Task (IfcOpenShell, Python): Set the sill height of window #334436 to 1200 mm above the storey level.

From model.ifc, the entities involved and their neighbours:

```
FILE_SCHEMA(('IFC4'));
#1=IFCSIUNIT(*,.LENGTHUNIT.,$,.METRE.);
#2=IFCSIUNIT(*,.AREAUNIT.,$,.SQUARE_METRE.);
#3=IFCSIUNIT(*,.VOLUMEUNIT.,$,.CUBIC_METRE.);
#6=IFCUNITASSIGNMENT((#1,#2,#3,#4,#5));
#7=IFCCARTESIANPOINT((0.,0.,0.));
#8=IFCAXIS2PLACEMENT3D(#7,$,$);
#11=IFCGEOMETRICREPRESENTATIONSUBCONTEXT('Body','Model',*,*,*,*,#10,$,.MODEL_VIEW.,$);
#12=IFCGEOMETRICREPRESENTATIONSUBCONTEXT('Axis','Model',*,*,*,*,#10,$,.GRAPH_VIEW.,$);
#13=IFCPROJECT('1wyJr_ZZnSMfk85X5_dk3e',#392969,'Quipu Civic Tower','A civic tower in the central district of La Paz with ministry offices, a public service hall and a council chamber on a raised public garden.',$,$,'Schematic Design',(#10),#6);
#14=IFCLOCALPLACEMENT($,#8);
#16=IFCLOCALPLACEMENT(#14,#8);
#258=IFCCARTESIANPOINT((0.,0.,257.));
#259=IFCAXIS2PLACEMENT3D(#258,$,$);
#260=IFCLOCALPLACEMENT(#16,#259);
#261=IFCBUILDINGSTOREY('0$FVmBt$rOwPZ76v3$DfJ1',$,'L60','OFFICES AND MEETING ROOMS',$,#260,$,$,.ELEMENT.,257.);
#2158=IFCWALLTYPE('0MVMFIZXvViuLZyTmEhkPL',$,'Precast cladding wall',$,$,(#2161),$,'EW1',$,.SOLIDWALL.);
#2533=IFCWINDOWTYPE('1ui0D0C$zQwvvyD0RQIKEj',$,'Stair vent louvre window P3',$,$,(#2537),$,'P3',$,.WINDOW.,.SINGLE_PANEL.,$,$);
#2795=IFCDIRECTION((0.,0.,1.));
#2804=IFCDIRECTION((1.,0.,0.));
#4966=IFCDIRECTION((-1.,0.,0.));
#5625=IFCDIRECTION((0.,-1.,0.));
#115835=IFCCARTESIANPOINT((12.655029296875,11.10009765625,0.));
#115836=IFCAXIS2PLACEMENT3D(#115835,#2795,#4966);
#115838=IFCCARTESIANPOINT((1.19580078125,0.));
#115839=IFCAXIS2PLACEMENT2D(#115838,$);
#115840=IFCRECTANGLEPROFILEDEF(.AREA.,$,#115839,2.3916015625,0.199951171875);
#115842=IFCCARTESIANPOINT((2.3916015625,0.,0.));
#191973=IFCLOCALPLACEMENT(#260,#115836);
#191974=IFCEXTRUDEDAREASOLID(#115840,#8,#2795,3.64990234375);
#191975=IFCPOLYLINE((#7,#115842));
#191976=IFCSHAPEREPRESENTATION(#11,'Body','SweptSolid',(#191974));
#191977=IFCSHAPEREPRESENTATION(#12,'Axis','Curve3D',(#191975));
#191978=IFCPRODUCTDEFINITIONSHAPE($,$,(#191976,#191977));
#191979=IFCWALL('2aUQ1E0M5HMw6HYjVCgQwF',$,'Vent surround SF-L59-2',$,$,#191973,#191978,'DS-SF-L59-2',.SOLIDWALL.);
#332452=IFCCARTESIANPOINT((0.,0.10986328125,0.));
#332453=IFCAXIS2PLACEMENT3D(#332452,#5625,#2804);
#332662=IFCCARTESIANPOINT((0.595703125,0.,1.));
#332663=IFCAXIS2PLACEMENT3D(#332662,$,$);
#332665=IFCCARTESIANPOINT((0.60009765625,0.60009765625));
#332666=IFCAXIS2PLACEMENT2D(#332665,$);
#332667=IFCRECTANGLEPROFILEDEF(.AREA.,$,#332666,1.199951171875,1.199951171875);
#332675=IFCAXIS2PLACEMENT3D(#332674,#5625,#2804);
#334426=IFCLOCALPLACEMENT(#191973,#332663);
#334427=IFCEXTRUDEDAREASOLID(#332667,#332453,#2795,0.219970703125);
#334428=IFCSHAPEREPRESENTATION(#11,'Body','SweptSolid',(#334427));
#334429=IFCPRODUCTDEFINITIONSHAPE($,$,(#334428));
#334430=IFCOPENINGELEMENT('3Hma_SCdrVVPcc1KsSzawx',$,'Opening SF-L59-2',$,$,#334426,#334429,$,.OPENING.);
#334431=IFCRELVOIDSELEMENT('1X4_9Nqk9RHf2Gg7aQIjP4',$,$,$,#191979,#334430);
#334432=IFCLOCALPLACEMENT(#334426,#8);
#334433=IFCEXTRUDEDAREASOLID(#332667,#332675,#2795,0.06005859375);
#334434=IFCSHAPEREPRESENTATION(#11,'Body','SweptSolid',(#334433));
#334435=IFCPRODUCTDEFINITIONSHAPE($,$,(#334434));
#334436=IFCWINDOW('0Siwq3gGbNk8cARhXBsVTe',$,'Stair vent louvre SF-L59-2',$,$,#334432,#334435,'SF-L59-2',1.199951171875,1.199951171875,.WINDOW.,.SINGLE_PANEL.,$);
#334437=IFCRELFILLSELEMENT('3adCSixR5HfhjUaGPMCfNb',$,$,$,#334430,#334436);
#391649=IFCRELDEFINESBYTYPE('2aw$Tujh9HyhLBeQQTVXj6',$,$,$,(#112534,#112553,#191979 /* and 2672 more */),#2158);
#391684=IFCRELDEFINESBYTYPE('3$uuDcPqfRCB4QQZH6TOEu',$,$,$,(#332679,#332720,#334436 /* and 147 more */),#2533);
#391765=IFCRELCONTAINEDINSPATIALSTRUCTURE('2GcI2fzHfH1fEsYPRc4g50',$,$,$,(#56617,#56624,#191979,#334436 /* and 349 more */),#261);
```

```python
import numpy as np
import ifcopenshell
import ifcopenshell.api.geometry
import ifcopenshell.geom
import ifcopenshell.util.element
import ifcopenshell.util.placement
import ifcopenshell.util.shape
import ifcopenshell.util.unit

model = ifcopenshell.open("model.ifc")
unit_scale = ifcopenshell.util.unit.calculate_unit_scale(model)

window = model.by_guid("0Siwq3gGbNk8cARhXBsVTe")
opening = window.FillsVoids[0].RelatingOpeningElement
storey = ifcopenshell.util.element.get_container(window, ifc_class="IfcBuildingStorey")
level = ifcopenshell.util.placement.get_local_placement(storey.ObjectPlacement)[2, 3]

# The opening's origin need not be at the sill, so measure its lowest point.
shape = ifcopenshell.geom.create_shape(ifcopenshell.geom.settings(), opening)
bottom = ifcopenshell.util.shape.get_shape_bottom_elevation(shape, shape.geometry) / unit_scale
dz = level + 1.2 / unit_scale - bottom

shift = np.array([0.0, 0.0, dz])
# The window is placed relative to its opening, so it follows when the opening moves.
matrix = ifcopenshell.util.placement.get_local_placement(opening.ObjectPlacement)
matrix[:3, 3] += shift
ifcopenshell.api.geometry.edit_object_placement(
    model, product=opening, matrix=matrix, is_si=False, should_transform_children=True
)

print(f"moved by {dz * unit_scale:+.3f} m")

model.write("model_v2.ifc")
```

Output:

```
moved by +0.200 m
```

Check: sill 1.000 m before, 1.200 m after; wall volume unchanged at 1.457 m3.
